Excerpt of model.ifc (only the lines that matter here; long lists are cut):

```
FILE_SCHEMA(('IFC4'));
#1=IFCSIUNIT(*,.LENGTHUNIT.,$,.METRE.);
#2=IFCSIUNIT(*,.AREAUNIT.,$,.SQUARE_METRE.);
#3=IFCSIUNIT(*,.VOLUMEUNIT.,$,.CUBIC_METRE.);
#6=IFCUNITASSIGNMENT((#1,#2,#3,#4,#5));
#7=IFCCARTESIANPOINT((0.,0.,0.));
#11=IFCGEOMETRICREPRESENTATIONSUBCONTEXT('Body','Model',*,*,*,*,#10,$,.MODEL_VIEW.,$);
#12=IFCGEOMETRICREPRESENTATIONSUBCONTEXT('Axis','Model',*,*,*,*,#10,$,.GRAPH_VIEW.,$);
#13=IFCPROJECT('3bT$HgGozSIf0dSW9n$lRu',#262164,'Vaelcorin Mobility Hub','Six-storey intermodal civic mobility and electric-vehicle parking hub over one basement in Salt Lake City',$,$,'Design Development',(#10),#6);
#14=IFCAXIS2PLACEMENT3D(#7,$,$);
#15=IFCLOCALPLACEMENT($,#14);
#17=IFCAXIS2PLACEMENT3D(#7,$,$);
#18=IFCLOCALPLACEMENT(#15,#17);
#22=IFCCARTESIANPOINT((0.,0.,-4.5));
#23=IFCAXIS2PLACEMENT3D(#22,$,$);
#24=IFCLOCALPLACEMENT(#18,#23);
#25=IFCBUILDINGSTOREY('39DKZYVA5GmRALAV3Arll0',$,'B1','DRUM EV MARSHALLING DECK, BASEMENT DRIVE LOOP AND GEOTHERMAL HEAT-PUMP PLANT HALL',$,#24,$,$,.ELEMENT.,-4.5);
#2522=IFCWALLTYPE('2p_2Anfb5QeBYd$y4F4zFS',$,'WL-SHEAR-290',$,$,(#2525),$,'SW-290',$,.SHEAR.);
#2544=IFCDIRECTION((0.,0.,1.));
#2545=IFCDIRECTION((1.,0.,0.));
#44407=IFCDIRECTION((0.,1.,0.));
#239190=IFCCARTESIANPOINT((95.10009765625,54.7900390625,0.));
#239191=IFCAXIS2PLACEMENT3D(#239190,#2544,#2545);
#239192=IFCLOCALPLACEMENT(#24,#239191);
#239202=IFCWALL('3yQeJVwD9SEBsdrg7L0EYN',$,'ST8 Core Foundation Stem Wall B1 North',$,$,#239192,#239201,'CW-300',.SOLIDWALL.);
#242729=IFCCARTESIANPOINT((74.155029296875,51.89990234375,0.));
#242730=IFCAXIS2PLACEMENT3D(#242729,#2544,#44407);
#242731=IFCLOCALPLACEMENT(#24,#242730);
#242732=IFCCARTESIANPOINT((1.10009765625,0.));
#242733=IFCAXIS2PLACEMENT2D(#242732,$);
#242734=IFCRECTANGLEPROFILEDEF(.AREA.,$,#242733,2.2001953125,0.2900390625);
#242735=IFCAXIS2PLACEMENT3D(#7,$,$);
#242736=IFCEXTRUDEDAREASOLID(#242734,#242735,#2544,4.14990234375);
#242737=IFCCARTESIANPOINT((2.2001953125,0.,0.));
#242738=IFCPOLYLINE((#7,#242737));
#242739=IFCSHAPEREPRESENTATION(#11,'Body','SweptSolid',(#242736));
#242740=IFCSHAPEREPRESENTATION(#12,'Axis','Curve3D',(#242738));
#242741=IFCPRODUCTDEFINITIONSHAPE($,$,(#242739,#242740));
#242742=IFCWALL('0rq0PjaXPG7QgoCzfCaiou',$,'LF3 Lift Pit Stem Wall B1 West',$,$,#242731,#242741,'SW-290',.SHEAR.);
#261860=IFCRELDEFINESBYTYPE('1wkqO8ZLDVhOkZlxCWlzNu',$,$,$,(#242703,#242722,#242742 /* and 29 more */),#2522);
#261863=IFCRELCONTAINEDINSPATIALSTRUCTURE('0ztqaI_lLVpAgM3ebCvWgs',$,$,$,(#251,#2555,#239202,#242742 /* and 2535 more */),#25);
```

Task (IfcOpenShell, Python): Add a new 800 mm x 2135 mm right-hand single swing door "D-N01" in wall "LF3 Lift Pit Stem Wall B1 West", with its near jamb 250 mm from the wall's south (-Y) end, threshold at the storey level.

```python
import numpy as np
import ifcopenshell
import ifcopenshell.api.feature
import ifcopenshell.api.geometry
import ifcopenshell.api.root
import ifcopenshell.api.spatial
import ifcopenshell.geom
import ifcopenshell.util.element
import ifcopenshell.util.placement
import ifcopenshell.util.representation
import ifcopenshell.util.shape
import ifcopenshell.util.unit

model = ifcopenshell.open("model.ifc")
unit_scale = ifcopenshell.util.unit.calculate_unit_scale(model)
settings = ifcopenshell.geom.settings()


def volume(element):
    """Net volume in cubic metres, openings subtracted."""
    shape = ifcopenshell.geom.create_shape(settings, element)
    return ifcopenshell.util.shape.get_volume(shape.geometry)


wall = model.by_id(242742)
storey = ifcopenshell.util.element.get_container(wall, ifc_class="IfcBuildingStorey")
context = ifcopenshell.util.representation.get_context(model, "Model", "Body", "MODEL_VIEW")
before = volume(wall)

width, height, from_end, sill = 0.8, 2.135, 0.25, 0.0  # metres

# The wall runs along its own X axis, and the end named is its -X end.
wall_shape = ifcopenshell.geom.create_shape(settings, wall)
x, y, z = ifcopenshell.util.shape.get_vertices(wall_shape.geometry).T
start = x.min() + from_end
face, thickness = float(y.min()), float(y.max() - y.min())
wall_matrix = ifcopenshell.util.placement.get_local_placement(wall.ObjectPlacement)
level = ifcopenshell.util.placement.get_local_placement(storey.ObjectPlacement)[2, 3]


def in_wall(x, y):
    """Placement at x, y metres in the wall's axes, at sill height."""
    matrix = wall_matrix.copy()
    matrix[:, 3] = wall_matrix @ np.array([x / unit_scale, y / unit_scale, 0.0, 1.0])
    matrix[2, 3] = level + sill / unit_scale
    return matrix


# Opening: a box that overshoots both wall faces by 50 mm.
opening = ifcopenshell.api.root.create_entity(model, ifc_class="IfcOpeningElement", predefined_type="OPENING")
box = ifcopenshell.api.geometry.add_wall_representation(
    model, context=context, length=width, height=height, thickness=thickness + 0.1
)
ifcopenshell.api.geometry.assign_representation(model, product=opening, representation=box)
ifcopenshell.api.geometry.edit_object_placement(model, product=opening, matrix=in_wall(start, face - 0.05), is_si=False)
ifcopenshell.api.feature.add_feature(model, feature=opening, element=wall)

door = ifcopenshell.api.root.create_entity(model, ifc_class="IfcDoor", name="D-N01", predefined_type="DOOR")
door.OverallWidth, door.OverallHeight = width / unit_scale, height / unit_scale
door.OperationType = "SINGLE_SWING_RIGHT"
body = ifcopenshell.api.geometry.add_door_representation(
    model,
    context=context,
    overall_width=door.OverallWidth,
    overall_height=door.OverallHeight,
    operation_type="SINGLE_SWING_RIGHT",
    lining_properties={"LiningDepth": thickness / unit_scale, "ThresholdDepth": thickness / unit_scale},
)
ifcopenshell.api.geometry.assign_representation(model, product=door, representation=body)
ifcopenshell.api.spatial.assign_container(model, products=[door], relating_structure=storey)
ifcopenshell.api.feature.add_filling(model, opening=opening, element=door)

# The lining spans the wall, so the door starts at the wall face.
ifcopenshell.api.geometry.edit_object_placement(model, product=door, matrix=in_wall(start, face), is_si=False)

after = volume(wall)

print(f"wall volume {before:.3f} -> {after:.3f} m3")

model.write("model-out.ifc")
```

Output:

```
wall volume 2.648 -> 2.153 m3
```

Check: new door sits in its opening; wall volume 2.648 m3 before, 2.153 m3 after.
